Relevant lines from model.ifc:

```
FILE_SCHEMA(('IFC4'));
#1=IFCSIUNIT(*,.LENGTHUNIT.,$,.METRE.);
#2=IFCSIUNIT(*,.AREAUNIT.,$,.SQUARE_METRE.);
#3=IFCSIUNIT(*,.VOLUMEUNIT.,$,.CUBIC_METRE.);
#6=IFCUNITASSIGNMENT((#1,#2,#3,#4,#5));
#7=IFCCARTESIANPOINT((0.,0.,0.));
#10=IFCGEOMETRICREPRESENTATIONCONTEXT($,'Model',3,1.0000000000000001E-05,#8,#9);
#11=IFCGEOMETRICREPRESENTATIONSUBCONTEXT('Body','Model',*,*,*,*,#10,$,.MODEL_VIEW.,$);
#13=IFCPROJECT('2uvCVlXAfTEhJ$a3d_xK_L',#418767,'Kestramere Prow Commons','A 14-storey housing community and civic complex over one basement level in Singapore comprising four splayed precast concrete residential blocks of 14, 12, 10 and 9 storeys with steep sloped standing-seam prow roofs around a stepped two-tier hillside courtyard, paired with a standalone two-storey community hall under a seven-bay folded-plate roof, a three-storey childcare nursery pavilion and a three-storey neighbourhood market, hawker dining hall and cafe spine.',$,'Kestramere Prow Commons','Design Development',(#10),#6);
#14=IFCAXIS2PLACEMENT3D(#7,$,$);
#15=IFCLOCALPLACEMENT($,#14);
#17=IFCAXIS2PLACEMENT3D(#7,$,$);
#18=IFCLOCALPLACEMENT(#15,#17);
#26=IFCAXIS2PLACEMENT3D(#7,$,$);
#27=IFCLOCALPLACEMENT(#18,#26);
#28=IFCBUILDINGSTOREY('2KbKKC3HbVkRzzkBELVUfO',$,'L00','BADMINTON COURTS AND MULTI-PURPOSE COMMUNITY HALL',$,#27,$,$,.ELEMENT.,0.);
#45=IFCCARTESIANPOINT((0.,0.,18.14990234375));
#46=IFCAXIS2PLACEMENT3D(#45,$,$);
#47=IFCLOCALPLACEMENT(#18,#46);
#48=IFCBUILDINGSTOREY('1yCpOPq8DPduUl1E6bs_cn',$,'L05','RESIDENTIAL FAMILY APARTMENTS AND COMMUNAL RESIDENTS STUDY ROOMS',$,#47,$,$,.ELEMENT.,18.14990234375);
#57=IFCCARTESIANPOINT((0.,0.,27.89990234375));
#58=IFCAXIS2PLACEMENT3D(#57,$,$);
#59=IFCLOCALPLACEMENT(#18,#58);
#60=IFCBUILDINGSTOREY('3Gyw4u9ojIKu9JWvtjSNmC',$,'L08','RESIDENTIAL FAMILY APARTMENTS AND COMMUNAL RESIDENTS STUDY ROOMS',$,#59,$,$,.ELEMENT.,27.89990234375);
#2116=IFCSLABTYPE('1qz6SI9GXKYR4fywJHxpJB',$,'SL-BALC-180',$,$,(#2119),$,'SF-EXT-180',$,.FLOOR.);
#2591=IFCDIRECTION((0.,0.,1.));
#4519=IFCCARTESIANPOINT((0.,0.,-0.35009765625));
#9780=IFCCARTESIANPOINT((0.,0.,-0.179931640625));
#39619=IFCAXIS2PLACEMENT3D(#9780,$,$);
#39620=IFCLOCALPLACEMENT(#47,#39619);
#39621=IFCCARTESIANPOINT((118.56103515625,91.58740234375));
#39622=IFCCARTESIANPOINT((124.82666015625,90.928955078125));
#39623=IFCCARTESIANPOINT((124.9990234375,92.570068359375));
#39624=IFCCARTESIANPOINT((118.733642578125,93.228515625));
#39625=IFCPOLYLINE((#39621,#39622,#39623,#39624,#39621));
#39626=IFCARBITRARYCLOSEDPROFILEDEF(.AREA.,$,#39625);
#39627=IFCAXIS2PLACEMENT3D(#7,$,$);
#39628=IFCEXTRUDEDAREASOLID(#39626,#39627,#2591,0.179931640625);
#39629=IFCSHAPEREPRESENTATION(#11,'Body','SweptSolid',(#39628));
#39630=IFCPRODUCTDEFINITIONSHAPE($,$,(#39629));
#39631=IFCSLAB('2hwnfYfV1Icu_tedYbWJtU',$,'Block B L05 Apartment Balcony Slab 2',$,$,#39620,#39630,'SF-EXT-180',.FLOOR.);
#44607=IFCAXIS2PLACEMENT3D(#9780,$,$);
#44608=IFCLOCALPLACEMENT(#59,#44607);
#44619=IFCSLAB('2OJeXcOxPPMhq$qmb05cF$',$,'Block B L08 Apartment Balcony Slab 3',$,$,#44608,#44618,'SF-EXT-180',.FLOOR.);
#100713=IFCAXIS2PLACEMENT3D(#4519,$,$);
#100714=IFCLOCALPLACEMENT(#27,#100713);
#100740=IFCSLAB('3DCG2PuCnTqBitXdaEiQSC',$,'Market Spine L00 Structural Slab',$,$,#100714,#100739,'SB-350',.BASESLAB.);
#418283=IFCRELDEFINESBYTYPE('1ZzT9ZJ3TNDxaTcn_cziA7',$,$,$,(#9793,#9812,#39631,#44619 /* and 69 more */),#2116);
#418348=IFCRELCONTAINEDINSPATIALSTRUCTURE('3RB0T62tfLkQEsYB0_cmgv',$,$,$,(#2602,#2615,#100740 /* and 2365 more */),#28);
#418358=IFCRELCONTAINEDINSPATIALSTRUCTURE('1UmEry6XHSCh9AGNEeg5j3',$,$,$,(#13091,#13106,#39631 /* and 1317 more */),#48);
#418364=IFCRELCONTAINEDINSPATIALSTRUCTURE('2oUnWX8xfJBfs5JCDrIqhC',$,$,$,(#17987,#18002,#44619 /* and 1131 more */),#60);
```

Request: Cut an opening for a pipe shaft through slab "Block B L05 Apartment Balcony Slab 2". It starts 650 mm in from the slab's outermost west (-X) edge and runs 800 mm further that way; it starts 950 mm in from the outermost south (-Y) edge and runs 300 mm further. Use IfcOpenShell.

```python
import numpy as np
import ifcopenshell
import ifcopenshell.api.feature
import ifcopenshell.api.geometry
import ifcopenshell.api.root
import ifcopenshell.geom
import ifcopenshell.util.placement
import ifcopenshell.util.representation
import ifcopenshell.util.shape
import ifcopenshell.util.unit

model = ifcopenshell.open("model.ifc")
unit_scale = ifcopenshell.util.unit.calculate_unit_scale(model)
settings = ifcopenshell.geom.settings()


def volume(element):
    """Net volume in cubic metres, openings subtracted."""
    shape = ifcopenshell.geom.create_shape(settings, element)
    return ifcopenshell.util.shape.get_volume(shape.geometry)


slab = model.by_guid("2hwnfYfV1Icu_tedYbWJtU")
before = volume(slab)

# Extent in the slab's own axes, in metres. The edges named are its -X and -Y sides.
slab_shape = ifcopenshell.geom.create_shape(settings, slab)
vertices = ifcopenshell.util.shape.get_vertices(slab_shape.geometry)
x_min, y_min, bottom = vertices.min(axis=0)
top = vertices[:, 2].max()

opening = ifcopenshell.api.root.create_entity(model, ifc_class="IfcOpeningElement", name="Pipe shaft opening", predefined_type="OPENING")
context = ifcopenshell.util.representation.get_context(model, "Model", "Body", "MODEL_VIEW")
width, depth = 0.8, 0.3
outline = [(0.0, 0.0), (width, 0.0), (width, depth), (0.0, depth), (0.0, 0.0)]
# Overshoot both faces by 50 mm so the cut is clean.
shape = ifcopenshell.api.geometry.add_slab_representation(
    model, context=context, depth=top - bottom + 0.1, polyline=outline
)
ifcopenshell.api.geometry.assign_representation(model, product=opening, representation=shape)

matrix = ifcopenshell.util.placement.get_local_placement(slab.ObjectPlacement)
matrix[:, 3] = matrix @ np.append(np.array([x_min + 0.65, y_min + 0.95, bottom - 0.05]) / unit_scale, 1.0)
ifcopenshell.api.geometry.edit_object_placement(model, product=opening, matrix=matrix, is_si=False)
ifcopenshell.api.feature.add_feature(model, feature=opening, element=slab)

after = volume(slab)

print(f"slab volume {before:.3f} -> {after:.3f} m3")

model.write("model-out.ifc")
```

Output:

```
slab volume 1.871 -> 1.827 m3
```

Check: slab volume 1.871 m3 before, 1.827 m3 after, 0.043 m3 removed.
